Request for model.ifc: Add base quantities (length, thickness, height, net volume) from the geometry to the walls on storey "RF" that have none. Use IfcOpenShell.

First a look at what the model holds.

```python
import ifcopenshell
import ifcopenshell.util.element
import ifcopenshell.util.unit

model = ifcopenshell.open("model.ifc")
print(model.schema)
for unit_type in ("LENGTHUNIT", "AREAUNIT", "VOLUMEUNIT"):
    print(unit_type, ifcopenshell.util.unit.calculate_unit_scale(model, unit_type))
storey = next(s for s in model.by_type("IfcBuildingStorey") if s.Name == "RF")
walls = [e for e in ifcopenshell.util.element.get_decomposition(storey) if e.is_a("IfcWall")]
for e in sorted(walls, key=lambda e: e.id()):
    print(e.id(), e.is_a(), e.Name, list(ifcopenshell.util.element.get_psets(e, qtos_only=True)), sep=" | ")
```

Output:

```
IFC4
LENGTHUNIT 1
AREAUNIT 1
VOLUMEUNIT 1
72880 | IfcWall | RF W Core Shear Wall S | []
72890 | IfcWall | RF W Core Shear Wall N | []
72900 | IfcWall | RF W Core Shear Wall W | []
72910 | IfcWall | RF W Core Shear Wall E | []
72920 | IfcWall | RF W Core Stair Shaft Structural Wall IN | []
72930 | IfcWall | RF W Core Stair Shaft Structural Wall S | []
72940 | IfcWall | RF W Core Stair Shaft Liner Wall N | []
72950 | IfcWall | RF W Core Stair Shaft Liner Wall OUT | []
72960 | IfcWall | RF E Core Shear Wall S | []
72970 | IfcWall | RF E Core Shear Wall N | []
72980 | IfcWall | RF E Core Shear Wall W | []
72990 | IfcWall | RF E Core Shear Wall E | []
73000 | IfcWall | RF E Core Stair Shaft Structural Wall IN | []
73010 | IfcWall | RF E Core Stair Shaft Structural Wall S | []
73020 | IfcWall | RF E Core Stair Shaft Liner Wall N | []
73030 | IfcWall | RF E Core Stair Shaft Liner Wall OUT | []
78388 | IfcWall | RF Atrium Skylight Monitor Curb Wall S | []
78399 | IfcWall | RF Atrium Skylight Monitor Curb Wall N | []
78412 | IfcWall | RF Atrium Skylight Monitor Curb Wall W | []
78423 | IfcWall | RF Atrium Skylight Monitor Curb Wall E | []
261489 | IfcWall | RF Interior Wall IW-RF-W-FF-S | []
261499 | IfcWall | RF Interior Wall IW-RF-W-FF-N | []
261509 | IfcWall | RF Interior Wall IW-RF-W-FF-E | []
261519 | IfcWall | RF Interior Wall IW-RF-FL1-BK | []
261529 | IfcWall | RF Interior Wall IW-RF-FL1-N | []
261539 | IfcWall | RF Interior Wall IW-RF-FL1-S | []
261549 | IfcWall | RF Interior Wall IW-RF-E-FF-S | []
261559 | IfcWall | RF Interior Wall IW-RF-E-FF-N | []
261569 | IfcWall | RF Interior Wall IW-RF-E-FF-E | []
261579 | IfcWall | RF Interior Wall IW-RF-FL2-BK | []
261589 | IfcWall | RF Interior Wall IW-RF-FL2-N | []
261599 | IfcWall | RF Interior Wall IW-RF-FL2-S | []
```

```python
import ifcopenshell
import ifcopenshell.api.pset
import ifcopenshell.geom
import ifcopenshell.util.element
import ifcopenshell.util.shape
import ifcopenshell.util.unit

model = ifcopenshell.open("model.ifc")
unit_scale = ifcopenshell.util.unit.calculate_unit_scale(model)
volume_scale = ifcopenshell.util.unit.calculate_unit_scale(model, "VOLUMEUNIT")
settings = ifcopenshell.geom.settings()

storey = next(s for s in model.by_type("IfcBuildingStorey") if s.Name == "RF")
walls = [e for e in ifcopenshell.util.element.get_decomposition(storey) if e.is_a("IfcWall")]

for e in sorted(walls, key=lambda e: e.id()):
    if ifcopenshell.util.element.get_psets(e, qtos_only=True, should_inherit=False):
        continue
    # Geometry comes back in metres, in the element's own axes.
    shape = ifcopenshell.geom.create_shape(settings, e)
    values = {
        "Length": ifcopenshell.util.shape.get_x(shape.geometry) / unit_scale,
        "Width": ifcopenshell.util.shape.get_y(shape.geometry) / unit_scale,
        "Height": ifcopenshell.util.shape.get_z(shape.geometry) / unit_scale,
        "NetVolume": ifcopenshell.util.shape.get_volume(shape.geometry) / volume_scale,
    }
    qto = ifcopenshell.api.pset.add_qto(model, product=e, name="Qto_WallBaseQuantities")
    ifcopenshell.api.pset.edit_qto(model, qto=qto, properties=values)
    print(e.id(), {k: round(v, 3) for k, v in values.items()})

model.write("model_v2.ifc")
```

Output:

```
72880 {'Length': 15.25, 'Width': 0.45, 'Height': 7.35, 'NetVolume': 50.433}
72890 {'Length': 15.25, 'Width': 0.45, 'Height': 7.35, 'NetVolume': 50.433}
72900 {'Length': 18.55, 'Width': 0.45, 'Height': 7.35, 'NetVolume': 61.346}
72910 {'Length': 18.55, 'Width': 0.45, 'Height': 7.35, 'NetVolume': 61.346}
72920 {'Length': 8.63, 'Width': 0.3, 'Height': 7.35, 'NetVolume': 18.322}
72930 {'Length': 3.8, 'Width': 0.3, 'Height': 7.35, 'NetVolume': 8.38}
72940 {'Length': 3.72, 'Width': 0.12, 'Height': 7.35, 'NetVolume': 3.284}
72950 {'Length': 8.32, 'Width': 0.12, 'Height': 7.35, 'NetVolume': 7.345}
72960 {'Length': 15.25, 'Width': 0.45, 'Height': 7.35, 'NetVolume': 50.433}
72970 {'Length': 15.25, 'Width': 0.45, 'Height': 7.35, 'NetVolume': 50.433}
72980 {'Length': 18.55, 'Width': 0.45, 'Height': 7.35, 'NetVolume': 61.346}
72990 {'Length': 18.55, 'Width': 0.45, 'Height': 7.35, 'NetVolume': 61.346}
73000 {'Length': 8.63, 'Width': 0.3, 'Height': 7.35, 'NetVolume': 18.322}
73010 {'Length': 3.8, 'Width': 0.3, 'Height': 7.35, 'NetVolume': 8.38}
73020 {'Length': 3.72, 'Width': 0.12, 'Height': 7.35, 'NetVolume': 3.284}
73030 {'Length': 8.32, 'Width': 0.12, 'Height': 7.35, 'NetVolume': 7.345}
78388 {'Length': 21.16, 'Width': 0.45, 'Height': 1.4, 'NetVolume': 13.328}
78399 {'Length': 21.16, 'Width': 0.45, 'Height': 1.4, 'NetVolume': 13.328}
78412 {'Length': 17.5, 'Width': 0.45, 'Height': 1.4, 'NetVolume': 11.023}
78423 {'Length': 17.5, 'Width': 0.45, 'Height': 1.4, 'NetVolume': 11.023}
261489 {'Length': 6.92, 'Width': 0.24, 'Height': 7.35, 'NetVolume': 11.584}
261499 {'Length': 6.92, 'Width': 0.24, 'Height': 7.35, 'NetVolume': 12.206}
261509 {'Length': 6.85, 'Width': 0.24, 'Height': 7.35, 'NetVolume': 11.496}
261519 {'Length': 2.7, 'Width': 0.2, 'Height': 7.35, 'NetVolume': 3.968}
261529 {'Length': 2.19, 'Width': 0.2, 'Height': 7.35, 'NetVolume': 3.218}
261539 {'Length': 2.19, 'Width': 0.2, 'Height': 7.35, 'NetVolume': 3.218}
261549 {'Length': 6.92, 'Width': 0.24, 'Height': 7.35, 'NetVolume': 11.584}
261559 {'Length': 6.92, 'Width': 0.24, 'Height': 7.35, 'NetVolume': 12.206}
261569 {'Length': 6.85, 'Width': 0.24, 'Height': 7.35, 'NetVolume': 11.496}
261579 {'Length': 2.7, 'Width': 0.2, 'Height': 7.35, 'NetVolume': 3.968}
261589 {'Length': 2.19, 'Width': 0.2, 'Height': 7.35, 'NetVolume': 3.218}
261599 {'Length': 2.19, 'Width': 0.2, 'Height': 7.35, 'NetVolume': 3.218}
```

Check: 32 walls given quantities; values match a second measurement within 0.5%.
